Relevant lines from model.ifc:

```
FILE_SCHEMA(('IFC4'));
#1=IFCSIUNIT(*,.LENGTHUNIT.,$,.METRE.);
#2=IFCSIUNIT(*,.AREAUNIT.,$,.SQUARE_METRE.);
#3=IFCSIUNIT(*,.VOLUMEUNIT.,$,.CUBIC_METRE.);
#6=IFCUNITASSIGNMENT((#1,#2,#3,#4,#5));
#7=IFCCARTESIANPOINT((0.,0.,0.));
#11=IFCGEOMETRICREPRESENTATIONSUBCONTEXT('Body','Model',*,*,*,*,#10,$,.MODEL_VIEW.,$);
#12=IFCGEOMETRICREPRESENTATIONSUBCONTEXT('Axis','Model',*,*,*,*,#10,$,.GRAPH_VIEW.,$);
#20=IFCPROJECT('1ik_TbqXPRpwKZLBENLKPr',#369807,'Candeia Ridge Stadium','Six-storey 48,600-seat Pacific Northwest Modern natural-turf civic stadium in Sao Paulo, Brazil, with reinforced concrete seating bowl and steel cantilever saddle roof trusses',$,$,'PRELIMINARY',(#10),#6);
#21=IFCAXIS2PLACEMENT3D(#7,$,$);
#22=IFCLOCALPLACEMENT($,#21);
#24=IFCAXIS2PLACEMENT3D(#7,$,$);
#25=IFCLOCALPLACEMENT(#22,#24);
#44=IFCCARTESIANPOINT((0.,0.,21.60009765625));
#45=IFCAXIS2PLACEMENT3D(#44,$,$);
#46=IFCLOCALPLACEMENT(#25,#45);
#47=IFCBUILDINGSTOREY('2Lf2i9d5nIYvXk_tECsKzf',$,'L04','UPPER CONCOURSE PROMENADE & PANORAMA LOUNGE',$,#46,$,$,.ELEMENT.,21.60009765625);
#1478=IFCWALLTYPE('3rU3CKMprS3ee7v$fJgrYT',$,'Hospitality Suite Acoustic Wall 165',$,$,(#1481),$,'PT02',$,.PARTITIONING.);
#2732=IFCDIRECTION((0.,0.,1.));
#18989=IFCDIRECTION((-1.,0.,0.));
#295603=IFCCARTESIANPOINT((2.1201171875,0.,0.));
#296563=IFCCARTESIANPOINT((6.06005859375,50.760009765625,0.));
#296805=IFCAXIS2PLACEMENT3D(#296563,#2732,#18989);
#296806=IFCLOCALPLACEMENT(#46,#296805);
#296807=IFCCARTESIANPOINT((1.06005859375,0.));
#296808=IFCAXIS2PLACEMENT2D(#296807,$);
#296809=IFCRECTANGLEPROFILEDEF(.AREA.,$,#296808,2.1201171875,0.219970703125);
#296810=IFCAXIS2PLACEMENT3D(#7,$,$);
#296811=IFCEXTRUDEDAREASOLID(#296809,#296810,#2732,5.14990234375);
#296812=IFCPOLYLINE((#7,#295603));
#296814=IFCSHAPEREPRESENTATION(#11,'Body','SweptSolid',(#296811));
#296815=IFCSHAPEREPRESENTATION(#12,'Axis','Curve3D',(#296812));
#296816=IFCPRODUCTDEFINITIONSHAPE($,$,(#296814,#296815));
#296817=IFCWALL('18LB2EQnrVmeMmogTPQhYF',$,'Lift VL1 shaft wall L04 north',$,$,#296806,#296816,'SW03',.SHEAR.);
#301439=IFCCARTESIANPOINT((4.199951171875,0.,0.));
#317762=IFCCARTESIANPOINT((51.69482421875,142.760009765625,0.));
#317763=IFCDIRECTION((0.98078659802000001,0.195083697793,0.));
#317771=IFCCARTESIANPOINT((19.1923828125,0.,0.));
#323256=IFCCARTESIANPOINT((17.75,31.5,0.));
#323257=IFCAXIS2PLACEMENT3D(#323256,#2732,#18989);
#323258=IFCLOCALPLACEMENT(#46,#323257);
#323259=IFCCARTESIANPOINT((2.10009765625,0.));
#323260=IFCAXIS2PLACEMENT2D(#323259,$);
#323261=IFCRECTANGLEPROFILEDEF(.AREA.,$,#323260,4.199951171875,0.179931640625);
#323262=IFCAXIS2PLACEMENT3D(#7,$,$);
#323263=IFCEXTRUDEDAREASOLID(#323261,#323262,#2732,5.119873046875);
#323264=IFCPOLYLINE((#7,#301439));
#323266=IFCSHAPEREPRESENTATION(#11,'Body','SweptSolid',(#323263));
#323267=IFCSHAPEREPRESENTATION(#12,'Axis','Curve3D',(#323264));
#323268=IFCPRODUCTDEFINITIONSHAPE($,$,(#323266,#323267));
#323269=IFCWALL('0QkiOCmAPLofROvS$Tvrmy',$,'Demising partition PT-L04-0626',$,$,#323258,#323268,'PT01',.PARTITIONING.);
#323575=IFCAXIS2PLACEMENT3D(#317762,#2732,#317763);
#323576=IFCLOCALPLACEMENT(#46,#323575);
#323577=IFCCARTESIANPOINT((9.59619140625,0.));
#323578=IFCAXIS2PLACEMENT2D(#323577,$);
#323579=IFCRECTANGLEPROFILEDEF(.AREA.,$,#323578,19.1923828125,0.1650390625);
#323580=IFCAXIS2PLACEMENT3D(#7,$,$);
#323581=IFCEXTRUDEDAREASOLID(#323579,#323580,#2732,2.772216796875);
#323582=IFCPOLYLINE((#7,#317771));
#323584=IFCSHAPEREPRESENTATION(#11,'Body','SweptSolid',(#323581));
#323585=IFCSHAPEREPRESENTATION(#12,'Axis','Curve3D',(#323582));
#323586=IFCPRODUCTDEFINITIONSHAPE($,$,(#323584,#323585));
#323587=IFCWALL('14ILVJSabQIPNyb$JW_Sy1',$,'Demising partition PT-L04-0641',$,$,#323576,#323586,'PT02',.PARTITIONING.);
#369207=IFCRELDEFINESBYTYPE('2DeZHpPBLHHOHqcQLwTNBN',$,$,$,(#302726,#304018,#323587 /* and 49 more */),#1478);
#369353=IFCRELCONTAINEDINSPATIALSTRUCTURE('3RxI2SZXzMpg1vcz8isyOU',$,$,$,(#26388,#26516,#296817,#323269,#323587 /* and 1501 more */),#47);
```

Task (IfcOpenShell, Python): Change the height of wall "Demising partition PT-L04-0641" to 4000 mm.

```python
import ifcopenshell
import ifcopenshell.geom
import ifcopenshell.util.representation
import ifcopenshell.util.shape

model = ifcopenshell.open("model.ifc")
settings = ifcopenshell.geom.settings()


def volume(element):
    """Net volume in cubic metres, openings subtracted."""
    shape = ifcopenshell.geom.create_shape(settings, element)
    return ifcopenshell.util.shape.get_volume(shape.geometry)


wall = model.by_guid("14ILVJSabQIPNyb$JW_Sy1")
before = volume(wall)

body = ifcopenshell.util.representation.get_representation(wall, "Model", "Body")
solid = body.Items[0]
old_height = solid.Depth
solid.Depth = 4.0
after = volume(wall)

print(f"height {old_height:g} -> {solid.Depth:g}, volume {before:.3f} -> {after:.3f} m3")

model.write("model_rev.ifc")
```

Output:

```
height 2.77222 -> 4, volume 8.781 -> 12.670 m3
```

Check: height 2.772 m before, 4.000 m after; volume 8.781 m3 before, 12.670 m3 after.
